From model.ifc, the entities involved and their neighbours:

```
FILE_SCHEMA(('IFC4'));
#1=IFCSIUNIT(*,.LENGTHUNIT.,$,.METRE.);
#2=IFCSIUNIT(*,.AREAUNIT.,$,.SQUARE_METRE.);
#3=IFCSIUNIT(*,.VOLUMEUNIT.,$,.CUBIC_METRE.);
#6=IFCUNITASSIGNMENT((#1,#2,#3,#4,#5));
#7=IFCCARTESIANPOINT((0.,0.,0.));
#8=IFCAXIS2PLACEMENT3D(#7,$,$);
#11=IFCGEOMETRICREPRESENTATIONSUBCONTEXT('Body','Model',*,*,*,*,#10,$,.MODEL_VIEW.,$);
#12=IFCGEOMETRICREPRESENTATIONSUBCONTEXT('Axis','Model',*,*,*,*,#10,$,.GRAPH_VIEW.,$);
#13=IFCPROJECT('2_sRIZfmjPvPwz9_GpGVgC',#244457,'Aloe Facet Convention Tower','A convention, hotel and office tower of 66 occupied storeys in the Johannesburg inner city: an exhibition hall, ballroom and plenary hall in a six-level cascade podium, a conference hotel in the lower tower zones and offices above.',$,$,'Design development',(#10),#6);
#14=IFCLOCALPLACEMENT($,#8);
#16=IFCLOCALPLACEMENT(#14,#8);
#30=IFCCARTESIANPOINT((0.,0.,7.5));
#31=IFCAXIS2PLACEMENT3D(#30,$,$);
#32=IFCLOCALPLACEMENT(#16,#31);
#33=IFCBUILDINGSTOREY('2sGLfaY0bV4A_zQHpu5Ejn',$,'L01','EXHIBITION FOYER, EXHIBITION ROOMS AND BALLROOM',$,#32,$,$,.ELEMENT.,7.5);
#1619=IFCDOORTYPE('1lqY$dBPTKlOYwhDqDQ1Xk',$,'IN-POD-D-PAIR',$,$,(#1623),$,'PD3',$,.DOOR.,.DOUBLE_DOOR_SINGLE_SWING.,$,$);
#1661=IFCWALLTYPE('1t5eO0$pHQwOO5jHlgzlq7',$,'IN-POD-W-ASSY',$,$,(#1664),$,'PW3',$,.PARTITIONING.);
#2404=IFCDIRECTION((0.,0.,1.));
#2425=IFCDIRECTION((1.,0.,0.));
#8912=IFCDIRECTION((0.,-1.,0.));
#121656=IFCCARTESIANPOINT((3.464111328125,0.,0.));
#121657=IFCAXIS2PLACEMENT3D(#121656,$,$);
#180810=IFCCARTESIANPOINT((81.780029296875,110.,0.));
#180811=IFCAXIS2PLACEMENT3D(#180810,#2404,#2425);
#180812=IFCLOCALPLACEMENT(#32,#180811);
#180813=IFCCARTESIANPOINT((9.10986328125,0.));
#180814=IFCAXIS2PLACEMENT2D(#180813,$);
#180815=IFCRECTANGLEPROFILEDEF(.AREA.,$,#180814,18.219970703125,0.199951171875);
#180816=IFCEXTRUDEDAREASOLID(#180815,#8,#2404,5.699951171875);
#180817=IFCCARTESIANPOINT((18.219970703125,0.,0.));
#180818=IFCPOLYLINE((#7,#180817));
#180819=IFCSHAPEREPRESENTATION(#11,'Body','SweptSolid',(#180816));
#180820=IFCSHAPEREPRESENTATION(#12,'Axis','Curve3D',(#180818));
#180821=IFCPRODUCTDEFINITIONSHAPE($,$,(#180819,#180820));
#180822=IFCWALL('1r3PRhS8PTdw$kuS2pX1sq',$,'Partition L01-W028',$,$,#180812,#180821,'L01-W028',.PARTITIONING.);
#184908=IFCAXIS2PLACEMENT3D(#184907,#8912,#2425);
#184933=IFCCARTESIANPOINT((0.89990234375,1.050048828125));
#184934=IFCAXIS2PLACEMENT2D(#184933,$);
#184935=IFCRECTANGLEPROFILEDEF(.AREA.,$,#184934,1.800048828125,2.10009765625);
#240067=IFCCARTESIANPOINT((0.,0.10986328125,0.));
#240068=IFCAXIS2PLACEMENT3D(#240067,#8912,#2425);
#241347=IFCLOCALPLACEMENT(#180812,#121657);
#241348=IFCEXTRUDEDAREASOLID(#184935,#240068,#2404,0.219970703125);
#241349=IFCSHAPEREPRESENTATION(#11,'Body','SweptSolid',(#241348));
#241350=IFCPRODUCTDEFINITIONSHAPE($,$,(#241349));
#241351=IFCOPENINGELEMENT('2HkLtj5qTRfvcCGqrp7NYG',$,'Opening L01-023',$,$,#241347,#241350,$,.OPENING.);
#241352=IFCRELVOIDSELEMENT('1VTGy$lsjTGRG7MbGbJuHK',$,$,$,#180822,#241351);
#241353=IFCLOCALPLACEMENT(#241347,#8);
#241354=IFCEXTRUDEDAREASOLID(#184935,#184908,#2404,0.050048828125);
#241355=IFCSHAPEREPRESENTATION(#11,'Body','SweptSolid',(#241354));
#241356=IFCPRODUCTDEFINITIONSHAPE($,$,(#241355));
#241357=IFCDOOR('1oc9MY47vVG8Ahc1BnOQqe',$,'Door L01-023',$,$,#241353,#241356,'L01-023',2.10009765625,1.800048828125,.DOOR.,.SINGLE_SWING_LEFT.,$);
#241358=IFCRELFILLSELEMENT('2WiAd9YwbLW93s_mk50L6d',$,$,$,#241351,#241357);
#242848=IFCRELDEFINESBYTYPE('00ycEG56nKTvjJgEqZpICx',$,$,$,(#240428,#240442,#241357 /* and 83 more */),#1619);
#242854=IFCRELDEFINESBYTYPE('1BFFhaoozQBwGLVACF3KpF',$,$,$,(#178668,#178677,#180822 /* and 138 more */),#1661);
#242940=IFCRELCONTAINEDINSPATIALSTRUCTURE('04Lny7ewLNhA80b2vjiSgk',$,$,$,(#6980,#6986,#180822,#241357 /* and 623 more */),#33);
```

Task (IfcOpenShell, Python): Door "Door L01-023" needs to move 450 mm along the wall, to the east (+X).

```python
import ifcopenshell
import ifcopenshell.api.geometry
import ifcopenshell.util.placement
import ifcopenshell.util.unit

model = ifcopenshell.open("model.ifc")
unit_scale = ifcopenshell.util.unit.calculate_unit_scale(model)

door = model.by_guid("1oc9MY47vVG8Ahc1BnOQqe")
opening = door.FillsVoids[0].RelatingOpeningElement
wall = opening.VoidsElements[0].RelatingBuildingElement

wall_matrix = ifcopenshell.util.placement.get_local_placement(wall.ObjectPlacement)
shift = wall_matrix[:3, 0] * 0.45 / unit_scale
before = ifcopenshell.util.placement.get_local_placement(door.ObjectPlacement)[:3, 3].copy()

# The door is placed relative to its opening, so it follows when the opening moves.
matrix = ifcopenshell.util.placement.get_local_placement(opening.ObjectPlacement)
matrix[:3, 3] += shift
ifcopenshell.api.geometry.edit_object_placement(
    model, product=opening, matrix=matrix, is_si=False, should_transform_children=True
)

after = ifcopenshell.util.placement.get_local_placement(door.ObjectPlacement)[:3, 3]
print("door moved by", (after - before).round(3) + 0.0)

model.write("model_edited.ifc")
```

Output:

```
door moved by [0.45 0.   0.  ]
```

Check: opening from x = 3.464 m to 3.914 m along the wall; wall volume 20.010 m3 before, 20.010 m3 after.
